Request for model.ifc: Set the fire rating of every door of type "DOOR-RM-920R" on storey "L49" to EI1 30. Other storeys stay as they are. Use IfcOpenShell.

First a look at what the model holds.

```python
import ifcopenshell
import ifcopenshell.util.element

model = ifcopenshell.open("model.ifc")
print(model.schema)
storey = next(s for s in model.by_type("IfcBuildingStorey") if s.Name == "L49")
doors = [e for e in ifcopenshell.util.element.get_decomposition(storey) if e.is_a("IfcDoor")]
seen = {}
for e in doors:
    element_type = ifcopenshell.util.element.get_type(e)
    key = (element_type.Name if element_type != e and element_type else None, ifcopenshell.util.element.get_pset(e, "Pset_DoorCommon", "FireRating"))
    seen[key] = seen.get(key, 0) + 1
for (name, value), count in sorted(seen.items(), key=str):
    print(count, "x", name, "|", value)
```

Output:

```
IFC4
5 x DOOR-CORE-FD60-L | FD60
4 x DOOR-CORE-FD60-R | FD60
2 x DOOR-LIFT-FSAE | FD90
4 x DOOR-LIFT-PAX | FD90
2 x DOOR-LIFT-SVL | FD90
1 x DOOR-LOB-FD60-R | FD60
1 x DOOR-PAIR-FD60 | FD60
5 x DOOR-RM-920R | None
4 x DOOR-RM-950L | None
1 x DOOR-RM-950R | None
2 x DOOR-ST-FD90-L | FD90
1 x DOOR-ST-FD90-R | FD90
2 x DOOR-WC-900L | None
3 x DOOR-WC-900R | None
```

```python
import ifcopenshell
import ifcopenshell.api.pset
import ifcopenshell.util.element

model = ifcopenshell.open("model.ifc")

storey = next(s for s in model.by_type("IfcBuildingStorey") if s.Name == "L49")
doors = [e for e in ifcopenshell.util.element.get_decomposition(storey) if e.is_a("IfcDoor")]

count = 0
for e in doors:
    element_type = ifcopenshell.util.element.get_type(e)
    if element_type in (None, e) or element_type.Name != "DOOR-RM-920R":
        continue
    found = ifcopenshell.util.element.get_pset(e, "Pset_DoorCommon", should_inherit=False)
    if found:
        pset = model.by_id(found["id"])
        if len(ifcopenshell.util.element.get_elements_by_pset(pset)) > 1:
            pset = ifcopenshell.api.pset.unshare_pset(model, products=[e], pset=pset)[0]
    else:
        pset = ifcopenshell.api.pset.add_pset(model, product=e, name="Pset_DoorCommon")
    ifcopenshell.api.pset.edit_pset(model, pset=pset, properties={"FireRating": "EI1 30"})
    count += 1

print(count, "doors updated")

model.write("model_v2.ifc")
```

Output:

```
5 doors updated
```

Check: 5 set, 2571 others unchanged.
